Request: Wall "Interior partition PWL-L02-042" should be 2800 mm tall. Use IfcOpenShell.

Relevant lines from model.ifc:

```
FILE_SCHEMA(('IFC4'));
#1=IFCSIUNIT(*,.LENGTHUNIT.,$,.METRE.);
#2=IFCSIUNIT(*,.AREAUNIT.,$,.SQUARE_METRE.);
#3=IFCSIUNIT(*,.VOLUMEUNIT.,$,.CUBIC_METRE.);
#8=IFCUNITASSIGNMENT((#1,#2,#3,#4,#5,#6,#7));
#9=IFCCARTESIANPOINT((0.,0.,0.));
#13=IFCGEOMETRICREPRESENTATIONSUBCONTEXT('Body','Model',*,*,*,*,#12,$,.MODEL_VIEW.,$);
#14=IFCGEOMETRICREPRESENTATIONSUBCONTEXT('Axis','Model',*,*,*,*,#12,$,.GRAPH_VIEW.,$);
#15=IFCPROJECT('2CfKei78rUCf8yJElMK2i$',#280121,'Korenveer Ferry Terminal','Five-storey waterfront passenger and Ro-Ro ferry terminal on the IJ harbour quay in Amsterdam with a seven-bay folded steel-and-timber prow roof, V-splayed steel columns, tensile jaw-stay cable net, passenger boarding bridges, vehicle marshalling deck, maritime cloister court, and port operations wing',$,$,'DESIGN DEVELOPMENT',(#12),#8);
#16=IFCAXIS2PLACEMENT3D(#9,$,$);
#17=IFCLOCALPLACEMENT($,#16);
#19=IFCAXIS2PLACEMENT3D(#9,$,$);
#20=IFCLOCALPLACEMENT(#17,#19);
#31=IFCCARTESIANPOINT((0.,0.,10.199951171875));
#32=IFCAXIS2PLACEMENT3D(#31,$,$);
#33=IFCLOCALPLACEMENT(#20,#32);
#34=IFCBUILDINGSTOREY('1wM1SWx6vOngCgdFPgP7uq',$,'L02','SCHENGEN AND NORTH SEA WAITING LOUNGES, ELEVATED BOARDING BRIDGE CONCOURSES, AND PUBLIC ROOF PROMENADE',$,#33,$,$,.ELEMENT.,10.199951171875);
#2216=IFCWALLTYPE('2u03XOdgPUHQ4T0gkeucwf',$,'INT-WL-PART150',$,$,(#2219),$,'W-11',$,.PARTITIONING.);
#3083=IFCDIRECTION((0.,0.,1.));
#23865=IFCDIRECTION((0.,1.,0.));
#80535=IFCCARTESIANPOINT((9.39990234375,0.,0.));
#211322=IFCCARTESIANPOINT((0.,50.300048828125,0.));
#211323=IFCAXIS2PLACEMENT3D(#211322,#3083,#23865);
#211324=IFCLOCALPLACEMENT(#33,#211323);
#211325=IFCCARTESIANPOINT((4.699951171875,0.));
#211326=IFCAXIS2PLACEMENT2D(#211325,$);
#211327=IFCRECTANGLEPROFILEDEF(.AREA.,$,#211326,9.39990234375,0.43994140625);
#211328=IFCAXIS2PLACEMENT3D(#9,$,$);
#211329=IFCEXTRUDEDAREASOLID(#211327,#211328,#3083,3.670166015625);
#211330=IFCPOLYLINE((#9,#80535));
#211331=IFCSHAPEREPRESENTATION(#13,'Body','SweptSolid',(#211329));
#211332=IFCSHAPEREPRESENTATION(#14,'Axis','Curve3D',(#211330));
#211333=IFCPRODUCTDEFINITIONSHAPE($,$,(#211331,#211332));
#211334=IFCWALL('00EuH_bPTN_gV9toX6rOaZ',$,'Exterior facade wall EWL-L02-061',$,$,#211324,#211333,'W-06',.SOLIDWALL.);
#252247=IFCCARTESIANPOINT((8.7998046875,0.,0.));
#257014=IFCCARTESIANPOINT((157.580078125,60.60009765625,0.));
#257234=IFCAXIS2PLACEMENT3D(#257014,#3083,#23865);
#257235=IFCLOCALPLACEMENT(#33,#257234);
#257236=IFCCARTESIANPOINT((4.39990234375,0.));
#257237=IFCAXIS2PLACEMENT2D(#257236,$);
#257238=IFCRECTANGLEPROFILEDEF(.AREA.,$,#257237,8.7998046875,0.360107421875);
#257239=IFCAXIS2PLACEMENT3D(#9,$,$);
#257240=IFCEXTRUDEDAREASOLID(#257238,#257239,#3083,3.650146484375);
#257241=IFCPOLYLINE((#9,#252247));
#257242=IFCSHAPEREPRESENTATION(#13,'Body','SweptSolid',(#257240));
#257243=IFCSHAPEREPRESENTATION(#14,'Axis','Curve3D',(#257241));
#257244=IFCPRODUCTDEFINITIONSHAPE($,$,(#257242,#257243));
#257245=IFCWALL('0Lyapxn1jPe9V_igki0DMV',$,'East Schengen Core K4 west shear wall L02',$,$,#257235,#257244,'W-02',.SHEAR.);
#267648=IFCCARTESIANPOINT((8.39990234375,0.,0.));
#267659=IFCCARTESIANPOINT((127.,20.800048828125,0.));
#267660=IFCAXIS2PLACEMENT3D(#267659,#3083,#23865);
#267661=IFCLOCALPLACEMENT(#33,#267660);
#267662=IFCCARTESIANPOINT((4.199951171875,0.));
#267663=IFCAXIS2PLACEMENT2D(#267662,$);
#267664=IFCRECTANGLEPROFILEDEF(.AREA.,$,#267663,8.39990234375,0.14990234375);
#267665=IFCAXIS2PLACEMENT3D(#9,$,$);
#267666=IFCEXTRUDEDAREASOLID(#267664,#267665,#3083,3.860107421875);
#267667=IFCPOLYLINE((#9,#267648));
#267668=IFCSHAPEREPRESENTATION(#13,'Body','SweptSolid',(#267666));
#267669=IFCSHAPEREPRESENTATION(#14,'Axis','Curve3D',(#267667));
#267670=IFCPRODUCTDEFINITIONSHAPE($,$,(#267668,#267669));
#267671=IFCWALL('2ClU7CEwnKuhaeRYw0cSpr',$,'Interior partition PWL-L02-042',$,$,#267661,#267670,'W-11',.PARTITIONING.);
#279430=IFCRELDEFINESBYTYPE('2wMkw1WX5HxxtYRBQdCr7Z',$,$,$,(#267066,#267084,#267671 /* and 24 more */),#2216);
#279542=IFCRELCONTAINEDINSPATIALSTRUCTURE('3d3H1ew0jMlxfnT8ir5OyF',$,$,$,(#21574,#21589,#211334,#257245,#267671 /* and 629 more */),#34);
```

```python
import ifcopenshell
import ifcopenshell.geom
import ifcopenshell.util.representation
import ifcopenshell.util.shape
import ifcopenshell.util.unit

model = ifcopenshell.open("model.ifc")
unit_scale = ifcopenshell.util.unit.calculate_unit_scale(model)
settings = ifcopenshell.geom.settings()


def volume(element):
    """Net volume in cubic metres, openings subtracted."""
    shape = ifcopenshell.geom.create_shape(settings, element)
    return ifcopenshell.util.shape.get_volume(shape.geometry)


wall = model.by_id(267671)
before = volume(wall)

body = ifcopenshell.util.representation.get_representation(wall, "Model", "Body")
solid = body.Items[0]
old_height = solid.Depth
solid.Depth = 2.8 / unit_scale
after = volume(wall)

print(f"height {old_height:g} -> {solid.Depth:g}, volume {before:.3f} -> {after:.3f} m3")

model.write("model_edited.ifc")
```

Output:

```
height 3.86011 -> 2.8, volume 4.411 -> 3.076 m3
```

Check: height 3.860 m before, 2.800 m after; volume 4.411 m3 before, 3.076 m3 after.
